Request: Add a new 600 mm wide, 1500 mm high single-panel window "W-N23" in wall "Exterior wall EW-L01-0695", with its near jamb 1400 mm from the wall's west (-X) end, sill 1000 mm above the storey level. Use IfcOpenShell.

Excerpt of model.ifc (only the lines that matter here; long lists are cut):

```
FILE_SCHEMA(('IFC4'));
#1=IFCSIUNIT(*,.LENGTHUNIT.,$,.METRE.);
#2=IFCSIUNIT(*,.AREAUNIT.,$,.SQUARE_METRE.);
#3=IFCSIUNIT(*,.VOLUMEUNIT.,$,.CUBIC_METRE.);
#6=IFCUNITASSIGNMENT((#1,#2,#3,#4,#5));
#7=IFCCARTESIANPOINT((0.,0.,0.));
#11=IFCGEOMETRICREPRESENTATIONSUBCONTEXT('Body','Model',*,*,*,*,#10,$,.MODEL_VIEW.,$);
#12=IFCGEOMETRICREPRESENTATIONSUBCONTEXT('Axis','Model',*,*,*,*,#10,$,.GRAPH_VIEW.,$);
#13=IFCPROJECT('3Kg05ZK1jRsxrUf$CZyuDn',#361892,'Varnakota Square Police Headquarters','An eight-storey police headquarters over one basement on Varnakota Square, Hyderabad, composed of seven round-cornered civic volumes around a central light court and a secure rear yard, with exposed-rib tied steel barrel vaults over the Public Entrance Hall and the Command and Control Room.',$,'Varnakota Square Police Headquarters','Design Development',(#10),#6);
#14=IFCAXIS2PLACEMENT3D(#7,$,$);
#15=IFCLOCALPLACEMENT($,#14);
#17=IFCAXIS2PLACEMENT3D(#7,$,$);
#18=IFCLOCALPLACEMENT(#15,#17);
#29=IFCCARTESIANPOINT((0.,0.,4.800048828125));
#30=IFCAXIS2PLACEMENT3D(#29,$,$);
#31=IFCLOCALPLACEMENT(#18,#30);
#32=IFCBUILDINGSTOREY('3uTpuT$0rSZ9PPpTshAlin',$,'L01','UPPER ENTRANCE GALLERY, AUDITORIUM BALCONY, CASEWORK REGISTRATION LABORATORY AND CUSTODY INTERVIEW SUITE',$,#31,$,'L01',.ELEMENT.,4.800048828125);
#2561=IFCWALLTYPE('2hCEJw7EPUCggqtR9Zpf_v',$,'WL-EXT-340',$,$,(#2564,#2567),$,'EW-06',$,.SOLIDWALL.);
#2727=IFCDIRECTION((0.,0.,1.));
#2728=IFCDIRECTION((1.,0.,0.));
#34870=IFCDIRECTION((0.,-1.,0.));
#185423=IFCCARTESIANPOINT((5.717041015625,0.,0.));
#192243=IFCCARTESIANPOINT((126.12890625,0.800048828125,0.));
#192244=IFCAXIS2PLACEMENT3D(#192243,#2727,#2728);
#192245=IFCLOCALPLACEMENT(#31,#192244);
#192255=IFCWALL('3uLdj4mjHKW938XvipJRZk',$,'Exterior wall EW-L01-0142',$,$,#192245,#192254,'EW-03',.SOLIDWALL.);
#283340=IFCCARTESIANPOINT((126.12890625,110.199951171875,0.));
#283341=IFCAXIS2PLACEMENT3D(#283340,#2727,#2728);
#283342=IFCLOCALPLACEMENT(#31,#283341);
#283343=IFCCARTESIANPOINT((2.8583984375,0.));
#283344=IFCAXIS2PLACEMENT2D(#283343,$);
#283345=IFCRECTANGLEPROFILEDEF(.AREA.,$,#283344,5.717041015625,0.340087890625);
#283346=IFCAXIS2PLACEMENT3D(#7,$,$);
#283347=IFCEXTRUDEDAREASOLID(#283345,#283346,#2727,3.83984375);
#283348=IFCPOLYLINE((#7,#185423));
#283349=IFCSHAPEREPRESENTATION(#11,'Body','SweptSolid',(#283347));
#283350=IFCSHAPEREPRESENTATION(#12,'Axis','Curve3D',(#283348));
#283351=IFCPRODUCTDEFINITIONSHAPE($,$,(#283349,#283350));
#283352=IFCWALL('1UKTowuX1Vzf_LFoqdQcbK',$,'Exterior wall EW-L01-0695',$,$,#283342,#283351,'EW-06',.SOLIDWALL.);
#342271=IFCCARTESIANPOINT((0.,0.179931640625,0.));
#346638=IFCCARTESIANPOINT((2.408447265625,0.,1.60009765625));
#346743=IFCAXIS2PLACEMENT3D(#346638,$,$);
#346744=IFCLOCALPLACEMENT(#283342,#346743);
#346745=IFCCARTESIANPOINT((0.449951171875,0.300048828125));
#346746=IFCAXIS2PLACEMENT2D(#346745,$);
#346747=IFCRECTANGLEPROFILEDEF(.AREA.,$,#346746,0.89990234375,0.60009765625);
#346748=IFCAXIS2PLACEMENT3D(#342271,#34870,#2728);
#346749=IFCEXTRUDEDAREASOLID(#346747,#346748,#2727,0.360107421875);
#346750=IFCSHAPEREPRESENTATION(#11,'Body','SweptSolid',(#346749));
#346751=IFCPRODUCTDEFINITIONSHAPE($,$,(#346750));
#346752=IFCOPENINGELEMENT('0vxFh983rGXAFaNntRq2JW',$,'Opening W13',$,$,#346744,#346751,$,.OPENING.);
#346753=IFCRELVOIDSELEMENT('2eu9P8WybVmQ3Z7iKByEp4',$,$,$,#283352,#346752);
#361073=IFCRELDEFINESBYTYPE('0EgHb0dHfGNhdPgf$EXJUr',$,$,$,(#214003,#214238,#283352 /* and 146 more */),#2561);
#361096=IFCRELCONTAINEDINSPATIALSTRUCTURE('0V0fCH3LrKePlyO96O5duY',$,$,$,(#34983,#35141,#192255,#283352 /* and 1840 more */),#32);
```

```python
import numpy as np
import ifcopenshell
import ifcopenshell.api.feature
import ifcopenshell.api.geometry
import ifcopenshell.api.root
import ifcopenshell.api.spatial
import ifcopenshell.geom
import ifcopenshell.util.element
import ifcopenshell.util.placement
import ifcopenshell.util.representation
import ifcopenshell.util.shape
import ifcopenshell.util.unit

model = ifcopenshell.open("model.ifc")
unit_scale = ifcopenshell.util.unit.calculate_unit_scale(model)
settings = ifcopenshell.geom.settings()


def volume(element):
    """Net volume in cubic metres, openings subtracted."""
    shape = ifcopenshell.geom.create_shape(settings, element)
    return ifcopenshell.util.shape.get_volume(shape.geometry)


wall = model.by_guid("1UKTowuX1Vzf_LFoqdQcbK")
storey = ifcopenshell.util.element.get_container(wall, ifc_class="IfcBuildingStorey")
context = ifcopenshell.util.representation.get_context(model, "Model", "Body", "MODEL_VIEW")
before = volume(wall)

width, height, from_end, sill = 0.6, 1.5, 1.4, 1  # metres

# The wall runs along its own X axis, and the end named is its -X end.
wall_shape = ifcopenshell.geom.create_shape(settings, wall)
x, y, z = ifcopenshell.util.shape.get_vertices(wall_shape.geometry).T
start = x.min() + from_end
face, thickness = float(y.min()), float(y.max() - y.min())
wall_matrix = ifcopenshell.util.placement.get_local_placement(wall.ObjectPlacement)
level = ifcopenshell.util.placement.get_local_placement(storey.ObjectPlacement)[2, 3]


def in_wall(x, y):
    """Placement at x, y metres in the wall's axes, at sill height."""
    matrix = wall_matrix.copy()
    matrix[:, 3] = wall_matrix @ np.array([x / unit_scale, y / unit_scale, 0.0, 1.0])
    matrix[2, 3] = level + sill / unit_scale
    return matrix


# Opening: a box that overshoots both wall faces by 50 mm.
opening = ifcopenshell.api.root.create_entity(model, ifc_class="IfcOpeningElement", predefined_type="OPENING")
box = ifcopenshell.api.geometry.add_wall_representation(
    model, context=context, length=width, height=height, thickness=thickness + 0.1
)
ifcopenshell.api.geometry.assign_representation(model, product=opening, representation=box)
ifcopenshell.api.geometry.edit_object_placement(model, product=opening, matrix=in_wall(start, face - 0.05), is_si=False)
ifcopenshell.api.feature.add_feature(model, feature=opening, element=wall)

window = ifcopenshell.api.root.create_entity(model, ifc_class="IfcWindow", name="W-N23", predefined_type="WINDOW")
window.OverallWidth, window.OverallHeight = width / unit_scale, height / unit_scale
window.PartitioningType = "SINGLE_PANEL"
body = ifcopenshell.api.geometry.add_window_representation(
    model,
    context=context,
    overall_width=window.OverallWidth,
    overall_height=window.OverallHeight,
    partition_type="SINGLE_PANEL",
)
ifcopenshell.api.geometry.assign_representation(model, product=window, representation=body)
ifcopenshell.api.spatial.assign_container(model, products=[window], relating_structure=storey)
ifcopenshell.api.feature.add_filling(model, opening=opening, element=window)

# Centre the window in the wall's thickness.
ifcopenshell.api.geometry.edit_object_placement(model, product=window, matrix=in_wall(start, face), is_si=False)
window_shape = ifcopenshell.geom.create_shape(settings, window)
depth = ifcopenshell.util.shape.get_vertices(window_shape.geometry)[:, 1]
offset = face + thickness / 2 - (depth.min() + depth.max()) / 2
ifcopenshell.api.geometry.edit_object_placement(model, product=window, matrix=in_wall(start, offset), is_si=False)

after = volume(wall)

print(f"wall volume {before:.3f} -> {after:.3f} m3")

model.write("model_v2.ifc")
```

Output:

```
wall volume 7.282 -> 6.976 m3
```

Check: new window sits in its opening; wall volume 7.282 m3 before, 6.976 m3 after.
